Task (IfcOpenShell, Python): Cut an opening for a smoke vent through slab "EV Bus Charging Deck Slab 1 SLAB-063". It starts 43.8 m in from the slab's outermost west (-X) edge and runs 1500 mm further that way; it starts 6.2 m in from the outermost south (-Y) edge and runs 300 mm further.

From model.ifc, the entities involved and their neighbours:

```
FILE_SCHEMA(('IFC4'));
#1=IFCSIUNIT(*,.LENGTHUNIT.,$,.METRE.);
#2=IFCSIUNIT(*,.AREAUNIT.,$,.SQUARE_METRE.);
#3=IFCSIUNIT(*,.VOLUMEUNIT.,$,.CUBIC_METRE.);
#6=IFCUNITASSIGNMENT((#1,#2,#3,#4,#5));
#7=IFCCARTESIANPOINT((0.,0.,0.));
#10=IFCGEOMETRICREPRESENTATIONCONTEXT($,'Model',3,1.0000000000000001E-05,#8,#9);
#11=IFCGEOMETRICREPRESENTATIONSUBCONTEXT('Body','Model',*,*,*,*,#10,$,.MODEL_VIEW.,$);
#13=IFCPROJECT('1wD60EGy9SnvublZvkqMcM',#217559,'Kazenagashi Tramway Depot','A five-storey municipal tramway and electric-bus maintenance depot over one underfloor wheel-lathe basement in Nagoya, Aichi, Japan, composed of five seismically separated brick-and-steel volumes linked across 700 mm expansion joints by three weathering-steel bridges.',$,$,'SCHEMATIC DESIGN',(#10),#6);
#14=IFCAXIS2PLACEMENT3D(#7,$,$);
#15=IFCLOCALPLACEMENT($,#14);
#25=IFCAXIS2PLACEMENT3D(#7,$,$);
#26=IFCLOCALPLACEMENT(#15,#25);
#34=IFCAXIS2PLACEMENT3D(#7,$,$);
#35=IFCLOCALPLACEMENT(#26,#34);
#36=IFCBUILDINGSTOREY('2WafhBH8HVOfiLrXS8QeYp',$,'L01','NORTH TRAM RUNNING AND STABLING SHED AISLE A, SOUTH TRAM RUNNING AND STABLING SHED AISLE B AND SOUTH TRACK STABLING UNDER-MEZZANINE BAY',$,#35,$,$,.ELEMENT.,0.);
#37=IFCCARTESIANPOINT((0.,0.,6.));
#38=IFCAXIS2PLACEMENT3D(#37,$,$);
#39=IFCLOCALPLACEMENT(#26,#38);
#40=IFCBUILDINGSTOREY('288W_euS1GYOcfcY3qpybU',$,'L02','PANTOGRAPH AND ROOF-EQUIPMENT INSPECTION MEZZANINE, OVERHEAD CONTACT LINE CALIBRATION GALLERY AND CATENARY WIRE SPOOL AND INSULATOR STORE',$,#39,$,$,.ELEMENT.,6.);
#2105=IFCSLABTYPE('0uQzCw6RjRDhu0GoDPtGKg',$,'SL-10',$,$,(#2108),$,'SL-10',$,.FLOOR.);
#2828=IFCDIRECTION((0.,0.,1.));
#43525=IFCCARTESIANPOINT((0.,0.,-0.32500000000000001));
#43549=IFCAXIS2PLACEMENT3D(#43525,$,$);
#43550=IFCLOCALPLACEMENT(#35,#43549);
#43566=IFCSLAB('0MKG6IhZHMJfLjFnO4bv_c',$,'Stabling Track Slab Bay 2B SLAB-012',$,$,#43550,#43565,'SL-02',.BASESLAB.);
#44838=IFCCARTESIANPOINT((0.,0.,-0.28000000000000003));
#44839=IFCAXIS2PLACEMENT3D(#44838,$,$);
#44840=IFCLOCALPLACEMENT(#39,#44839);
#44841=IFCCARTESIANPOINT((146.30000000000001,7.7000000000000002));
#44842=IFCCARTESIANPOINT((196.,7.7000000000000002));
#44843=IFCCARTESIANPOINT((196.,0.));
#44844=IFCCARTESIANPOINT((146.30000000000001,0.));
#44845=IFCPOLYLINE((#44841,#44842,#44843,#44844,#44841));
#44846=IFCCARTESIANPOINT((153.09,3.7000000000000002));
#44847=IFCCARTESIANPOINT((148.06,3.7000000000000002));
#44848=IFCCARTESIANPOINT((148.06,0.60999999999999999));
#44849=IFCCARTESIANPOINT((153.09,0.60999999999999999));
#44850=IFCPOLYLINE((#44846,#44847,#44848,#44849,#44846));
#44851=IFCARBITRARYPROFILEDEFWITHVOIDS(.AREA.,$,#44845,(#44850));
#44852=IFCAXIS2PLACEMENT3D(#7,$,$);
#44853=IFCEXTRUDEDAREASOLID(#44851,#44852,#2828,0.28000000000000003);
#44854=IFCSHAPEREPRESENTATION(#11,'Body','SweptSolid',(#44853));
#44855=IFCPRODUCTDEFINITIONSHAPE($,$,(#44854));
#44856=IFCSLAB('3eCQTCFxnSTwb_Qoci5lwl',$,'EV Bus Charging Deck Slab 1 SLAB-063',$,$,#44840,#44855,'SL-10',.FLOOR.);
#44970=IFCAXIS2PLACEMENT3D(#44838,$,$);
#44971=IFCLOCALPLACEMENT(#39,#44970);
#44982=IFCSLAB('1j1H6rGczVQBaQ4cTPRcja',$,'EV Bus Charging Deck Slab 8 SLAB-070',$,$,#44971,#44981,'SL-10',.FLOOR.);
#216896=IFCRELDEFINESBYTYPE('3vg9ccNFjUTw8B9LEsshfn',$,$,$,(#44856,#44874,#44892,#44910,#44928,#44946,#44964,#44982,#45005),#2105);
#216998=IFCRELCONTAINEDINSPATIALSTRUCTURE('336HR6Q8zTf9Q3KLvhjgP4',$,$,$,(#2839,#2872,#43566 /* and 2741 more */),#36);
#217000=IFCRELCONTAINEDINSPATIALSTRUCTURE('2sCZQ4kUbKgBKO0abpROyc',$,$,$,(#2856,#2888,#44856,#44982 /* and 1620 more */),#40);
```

```python
import numpy as np
import ifcopenshell
import ifcopenshell.api.feature
import ifcopenshell.api.geometry
import ifcopenshell.api.root
import ifcopenshell.geom
import ifcopenshell.util.placement
import ifcopenshell.util.representation
import ifcopenshell.util.shape
import ifcopenshell.util.unit

model = ifcopenshell.open("model.ifc")
unit_scale = ifcopenshell.util.unit.calculate_unit_scale(model)
settings = ifcopenshell.geom.settings()


def volume(element):
    """Net volume in cubic metres, openings subtracted."""
    shape = ifcopenshell.geom.create_shape(settings, element)
    return ifcopenshell.util.shape.get_volume(shape.geometry)


slab = model.by_guid("3eCQTCFxnSTwb_Qoci5lwl")
before = volume(slab)

# Extent in the slab's own axes, in metres. The edges named are its -X and -Y sides.
slab_shape = ifcopenshell.geom.create_shape(settings, slab)
vertices = ifcopenshell.util.shape.get_vertices(slab_shape.geometry)
x_min, y_min, bottom = vertices.min(axis=0)
top = vertices[:, 2].max()

opening = ifcopenshell.api.root.create_entity(model, ifc_class="IfcOpeningElement", name="Smoke vent opening", predefined_type="OPENING")
context = ifcopenshell.util.representation.get_context(model, "Model", "Body", "MODEL_VIEW")
width, depth = 1.5, 0.3
outline = [(0.0, 0.0), (width, 0.0), (width, depth), (0.0, depth), (0.0, 0.0)]
# Overshoot both faces by 50 mm so the cut is clean.
shape = ifcopenshell.api.geometry.add_slab_representation(
    model, context=context, depth=top - bottom + 0.1, polyline=outline
)
ifcopenshell.api.geometry.assign_representation(model, product=opening, representation=shape)

matrix = ifcopenshell.util.placement.get_local_placement(slab.ObjectPlacement)
matrix[:, 3] = matrix @ np.append(np.array([x_min + 43.8, y_min + 6.2, bottom - 0.05]) / unit_scale, 1.0)
ifcopenshell.api.geometry.edit_object_placement(model, product=opening, matrix=matrix, is_si=False)
ifcopenshell.api.feature.add_feature(model, feature=opening, element=slab)

after = volume(slab)

print(f"slab volume {before:.3f} -> {after:.3f} m3")

model.write("model-out.ifc")
```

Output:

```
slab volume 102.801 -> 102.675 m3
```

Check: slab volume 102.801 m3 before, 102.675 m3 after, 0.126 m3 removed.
